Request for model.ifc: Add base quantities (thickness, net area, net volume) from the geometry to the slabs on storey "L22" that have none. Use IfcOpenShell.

First a look at what the model holds.

```python
import ifcopenshell
import ifcopenshell.util.element
import ifcopenshell.util.unit

model = ifcopenshell.open("model.ifc")
print(model.schema)
for unit_type in ("LENGTHUNIT", "AREAUNIT", "VOLUMEUNIT"):
    print(unit_type, ifcopenshell.util.unit.calculate_unit_scale(model, unit_type))
storey = next(s for s in model.by_type("IfcBuildingStorey") if s.Name == "L22")
slabs = [e for e in ifcopenshell.util.element.get_decomposition(storey) if e.is_a("IfcSlab")]
for e in sorted(slabs, key=lambda e: e.id()):
    print(e.id(), e.is_a(), e.Name, list(ifcopenshell.util.element.get_psets(e, qtos_only=True)), sep=" | ")
```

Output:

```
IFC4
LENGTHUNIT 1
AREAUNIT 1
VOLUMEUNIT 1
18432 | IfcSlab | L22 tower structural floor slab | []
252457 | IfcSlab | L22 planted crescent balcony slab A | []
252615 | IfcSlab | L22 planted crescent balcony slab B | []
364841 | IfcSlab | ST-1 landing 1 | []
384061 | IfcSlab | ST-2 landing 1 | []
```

```python
import ifcopenshell
import ifcopenshell.api.pset
import ifcopenshell.geom
import ifcopenshell.util.element
import ifcopenshell.util.shape
import ifcopenshell.util.unit

model = ifcopenshell.open("model.ifc")
unit_scale = ifcopenshell.util.unit.calculate_unit_scale(model)
area_scale = ifcopenshell.util.unit.calculate_unit_scale(model, "AREAUNIT")
volume_scale = ifcopenshell.util.unit.calculate_unit_scale(model, "VOLUMEUNIT")
settings = ifcopenshell.geom.settings()

storey = next(s for s in model.by_type("IfcBuildingStorey") if s.Name == "L22")
slabs = [e for e in ifcopenshell.util.element.get_decomposition(storey) if e.is_a("IfcSlab")]

for e in sorted(slabs, key=lambda e: e.id()):
    if ifcopenshell.util.element.get_psets(e, qtos_only=True, should_inherit=False):
        continue
    # Geometry comes back in metres, in the element's own axes.
    shape = ifcopenshell.geom.create_shape(settings, e)
    values = {
        "Width": ifcopenshell.util.shape.get_z(shape.geometry) / unit_scale,
        "NetArea": ifcopenshell.util.shape.get_footprint_area(shape.geometry) / area_scale,
        "NetVolume": ifcopenshell.util.shape.get_volume(shape.geometry) / volume_scale,
    }
    qto = ifcopenshell.api.pset.add_qto(model, product=e, name="Qto_SlabBaseQuantities")
    ifcopenshell.api.pset.edit_qto(model, qto=qto, properties=values)
    print(e.id(), {k: round(v, 3) for k, v in values.items()})

model.write("model_edited.ifc")
```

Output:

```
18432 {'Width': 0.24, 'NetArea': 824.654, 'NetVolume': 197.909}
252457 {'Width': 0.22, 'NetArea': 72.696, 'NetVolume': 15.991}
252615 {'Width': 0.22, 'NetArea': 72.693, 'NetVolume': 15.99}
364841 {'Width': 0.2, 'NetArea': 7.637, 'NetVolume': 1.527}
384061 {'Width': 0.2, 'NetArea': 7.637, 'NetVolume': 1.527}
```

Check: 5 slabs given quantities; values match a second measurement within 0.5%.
